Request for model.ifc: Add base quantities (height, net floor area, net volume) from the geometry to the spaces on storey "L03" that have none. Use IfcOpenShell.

First a look at what the model holds.

```python
import ifcopenshell
import ifcopenshell.util.element
import ifcopenshell.util.unit

model = ifcopenshell.open("model.ifc")
print(model.schema)
for unit_type in ("LENGTHUNIT", "AREAUNIT", "VOLUMEUNIT"):
    print(unit_type, ifcopenshell.util.unit.calculate_unit_scale(model, unit_type))
storey = next(s for s in model.by_type("IfcBuildingStorey") if s.Name == "L03")
spaces = [e for e in ifcopenshell.util.element.get_decomposition(storey) if e.is_a("IfcSpace")]
for e in sorted(spaces, key=lambda e: e.id()):
    print(e.id(), e.is_a(), e.Name, list(ifcopenshell.util.element.get_psets(e, qtos_only=True)), sep=" | ")
```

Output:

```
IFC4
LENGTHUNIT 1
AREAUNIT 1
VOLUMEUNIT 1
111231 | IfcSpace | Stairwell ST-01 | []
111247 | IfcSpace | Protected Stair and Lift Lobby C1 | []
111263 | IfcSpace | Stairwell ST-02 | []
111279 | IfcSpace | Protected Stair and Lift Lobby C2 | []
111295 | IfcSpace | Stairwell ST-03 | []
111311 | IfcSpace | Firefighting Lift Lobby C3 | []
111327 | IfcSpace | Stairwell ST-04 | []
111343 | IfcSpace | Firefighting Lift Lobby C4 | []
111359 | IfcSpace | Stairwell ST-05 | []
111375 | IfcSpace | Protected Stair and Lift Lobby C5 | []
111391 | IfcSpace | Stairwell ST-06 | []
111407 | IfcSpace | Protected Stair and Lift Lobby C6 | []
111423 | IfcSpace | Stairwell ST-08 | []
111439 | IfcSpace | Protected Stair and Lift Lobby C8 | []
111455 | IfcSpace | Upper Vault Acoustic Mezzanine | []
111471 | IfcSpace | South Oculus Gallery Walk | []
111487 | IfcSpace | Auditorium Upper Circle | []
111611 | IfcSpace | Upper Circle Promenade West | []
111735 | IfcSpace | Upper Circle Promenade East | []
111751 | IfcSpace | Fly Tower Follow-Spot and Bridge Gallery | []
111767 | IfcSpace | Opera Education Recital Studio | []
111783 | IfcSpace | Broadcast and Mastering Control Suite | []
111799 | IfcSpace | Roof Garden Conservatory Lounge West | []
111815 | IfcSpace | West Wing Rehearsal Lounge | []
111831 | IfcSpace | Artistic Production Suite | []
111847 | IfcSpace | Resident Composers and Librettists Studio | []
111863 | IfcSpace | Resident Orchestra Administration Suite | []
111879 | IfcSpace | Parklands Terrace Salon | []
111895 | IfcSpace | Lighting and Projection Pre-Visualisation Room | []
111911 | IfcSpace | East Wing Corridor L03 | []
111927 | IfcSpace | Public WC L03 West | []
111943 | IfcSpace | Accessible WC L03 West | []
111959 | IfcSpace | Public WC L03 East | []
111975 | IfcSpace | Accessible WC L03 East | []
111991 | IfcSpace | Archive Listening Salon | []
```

```python
import ifcopenshell
import ifcopenshell.api.pset
import ifcopenshell.geom
import ifcopenshell.util.element
import ifcopenshell.util.shape
import ifcopenshell.util.unit

model = ifcopenshell.open("model.ifc")
unit_scale = ifcopenshell.util.unit.calculate_unit_scale(model)
area_scale = ifcopenshell.util.unit.calculate_unit_scale(model, "AREAUNIT")
volume_scale = ifcopenshell.util.unit.calculate_unit_scale(model, "VOLUMEUNIT")
settings = ifcopenshell.geom.settings()

storey = next(s for s in model.by_type("IfcBuildingStorey") if s.Name == "L03")
spaces = [e for e in ifcopenshell.util.element.get_decomposition(storey) if e.is_a("IfcSpace")]

for e in sorted(spaces, key=lambda e: e.id()):
    if ifcopenshell.util.element.get_psets(e, qtos_only=True, should_inherit=False):
        continue
    # Geometry comes back in metres, in the element's own axes.
    shape = ifcopenshell.geom.create_shape(settings, e)
    values = {
        "Height": ifcopenshell.util.shape.get_z(shape.geometry) / unit_scale,
        "NetFloorArea": ifcopenshell.util.shape.get_footprint_area(shape.geometry) / area_scale,
        "NetVolume": ifcopenshell.util.shape.get_volume(shape.geometry) / volume_scale,
    }
    qto = ifcopenshell.api.pset.add_qto(model, product=e, name="Qto_SpaceBaseQuantities")
    ifcopenshell.api.pset.edit_qto(model, qto=qto, properties=values)
    print(e.id(), {k: round(v, 3) for k, v in values.items()})

model.write("model_rev.ifc")
```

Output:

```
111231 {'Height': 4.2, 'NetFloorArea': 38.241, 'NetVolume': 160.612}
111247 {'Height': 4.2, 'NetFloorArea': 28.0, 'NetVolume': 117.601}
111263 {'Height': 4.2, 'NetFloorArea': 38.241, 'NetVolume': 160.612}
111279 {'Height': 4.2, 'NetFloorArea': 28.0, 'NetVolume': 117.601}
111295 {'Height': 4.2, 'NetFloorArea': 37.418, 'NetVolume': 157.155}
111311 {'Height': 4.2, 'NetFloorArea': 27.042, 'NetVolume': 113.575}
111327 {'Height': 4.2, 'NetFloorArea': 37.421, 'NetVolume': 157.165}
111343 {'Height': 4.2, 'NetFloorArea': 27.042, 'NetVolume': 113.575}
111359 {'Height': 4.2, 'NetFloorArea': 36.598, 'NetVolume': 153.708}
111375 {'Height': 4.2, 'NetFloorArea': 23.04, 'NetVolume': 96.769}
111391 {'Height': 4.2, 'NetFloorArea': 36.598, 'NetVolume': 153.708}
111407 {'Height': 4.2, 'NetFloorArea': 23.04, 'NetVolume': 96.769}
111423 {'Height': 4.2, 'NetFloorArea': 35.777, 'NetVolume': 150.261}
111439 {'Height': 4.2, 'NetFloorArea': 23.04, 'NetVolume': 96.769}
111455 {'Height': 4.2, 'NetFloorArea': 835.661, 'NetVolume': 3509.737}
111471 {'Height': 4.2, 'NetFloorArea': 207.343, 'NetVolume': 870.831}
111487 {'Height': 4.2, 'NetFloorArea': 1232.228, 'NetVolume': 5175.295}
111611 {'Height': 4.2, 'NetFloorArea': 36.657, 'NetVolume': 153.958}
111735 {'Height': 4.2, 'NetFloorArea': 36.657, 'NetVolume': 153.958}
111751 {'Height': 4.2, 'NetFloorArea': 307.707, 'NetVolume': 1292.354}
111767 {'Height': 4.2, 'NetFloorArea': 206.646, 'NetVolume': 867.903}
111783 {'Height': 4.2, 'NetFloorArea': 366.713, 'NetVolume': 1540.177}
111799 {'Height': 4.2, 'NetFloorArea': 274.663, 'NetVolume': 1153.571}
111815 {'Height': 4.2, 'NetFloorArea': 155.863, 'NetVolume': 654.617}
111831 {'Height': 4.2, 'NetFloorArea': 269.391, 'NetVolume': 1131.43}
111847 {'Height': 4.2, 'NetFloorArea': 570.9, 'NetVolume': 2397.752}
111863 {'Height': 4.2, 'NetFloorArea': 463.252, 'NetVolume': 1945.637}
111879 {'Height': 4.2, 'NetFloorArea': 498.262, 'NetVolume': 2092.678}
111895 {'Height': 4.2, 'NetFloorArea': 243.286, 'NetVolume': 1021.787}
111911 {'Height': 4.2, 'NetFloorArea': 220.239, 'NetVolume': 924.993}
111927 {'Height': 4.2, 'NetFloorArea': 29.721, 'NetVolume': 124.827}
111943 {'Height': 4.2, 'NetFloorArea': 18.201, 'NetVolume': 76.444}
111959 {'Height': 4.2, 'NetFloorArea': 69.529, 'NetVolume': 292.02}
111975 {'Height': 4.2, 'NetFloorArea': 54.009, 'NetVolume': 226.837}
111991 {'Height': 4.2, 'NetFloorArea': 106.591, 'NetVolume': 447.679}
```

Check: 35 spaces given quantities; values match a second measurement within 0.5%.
